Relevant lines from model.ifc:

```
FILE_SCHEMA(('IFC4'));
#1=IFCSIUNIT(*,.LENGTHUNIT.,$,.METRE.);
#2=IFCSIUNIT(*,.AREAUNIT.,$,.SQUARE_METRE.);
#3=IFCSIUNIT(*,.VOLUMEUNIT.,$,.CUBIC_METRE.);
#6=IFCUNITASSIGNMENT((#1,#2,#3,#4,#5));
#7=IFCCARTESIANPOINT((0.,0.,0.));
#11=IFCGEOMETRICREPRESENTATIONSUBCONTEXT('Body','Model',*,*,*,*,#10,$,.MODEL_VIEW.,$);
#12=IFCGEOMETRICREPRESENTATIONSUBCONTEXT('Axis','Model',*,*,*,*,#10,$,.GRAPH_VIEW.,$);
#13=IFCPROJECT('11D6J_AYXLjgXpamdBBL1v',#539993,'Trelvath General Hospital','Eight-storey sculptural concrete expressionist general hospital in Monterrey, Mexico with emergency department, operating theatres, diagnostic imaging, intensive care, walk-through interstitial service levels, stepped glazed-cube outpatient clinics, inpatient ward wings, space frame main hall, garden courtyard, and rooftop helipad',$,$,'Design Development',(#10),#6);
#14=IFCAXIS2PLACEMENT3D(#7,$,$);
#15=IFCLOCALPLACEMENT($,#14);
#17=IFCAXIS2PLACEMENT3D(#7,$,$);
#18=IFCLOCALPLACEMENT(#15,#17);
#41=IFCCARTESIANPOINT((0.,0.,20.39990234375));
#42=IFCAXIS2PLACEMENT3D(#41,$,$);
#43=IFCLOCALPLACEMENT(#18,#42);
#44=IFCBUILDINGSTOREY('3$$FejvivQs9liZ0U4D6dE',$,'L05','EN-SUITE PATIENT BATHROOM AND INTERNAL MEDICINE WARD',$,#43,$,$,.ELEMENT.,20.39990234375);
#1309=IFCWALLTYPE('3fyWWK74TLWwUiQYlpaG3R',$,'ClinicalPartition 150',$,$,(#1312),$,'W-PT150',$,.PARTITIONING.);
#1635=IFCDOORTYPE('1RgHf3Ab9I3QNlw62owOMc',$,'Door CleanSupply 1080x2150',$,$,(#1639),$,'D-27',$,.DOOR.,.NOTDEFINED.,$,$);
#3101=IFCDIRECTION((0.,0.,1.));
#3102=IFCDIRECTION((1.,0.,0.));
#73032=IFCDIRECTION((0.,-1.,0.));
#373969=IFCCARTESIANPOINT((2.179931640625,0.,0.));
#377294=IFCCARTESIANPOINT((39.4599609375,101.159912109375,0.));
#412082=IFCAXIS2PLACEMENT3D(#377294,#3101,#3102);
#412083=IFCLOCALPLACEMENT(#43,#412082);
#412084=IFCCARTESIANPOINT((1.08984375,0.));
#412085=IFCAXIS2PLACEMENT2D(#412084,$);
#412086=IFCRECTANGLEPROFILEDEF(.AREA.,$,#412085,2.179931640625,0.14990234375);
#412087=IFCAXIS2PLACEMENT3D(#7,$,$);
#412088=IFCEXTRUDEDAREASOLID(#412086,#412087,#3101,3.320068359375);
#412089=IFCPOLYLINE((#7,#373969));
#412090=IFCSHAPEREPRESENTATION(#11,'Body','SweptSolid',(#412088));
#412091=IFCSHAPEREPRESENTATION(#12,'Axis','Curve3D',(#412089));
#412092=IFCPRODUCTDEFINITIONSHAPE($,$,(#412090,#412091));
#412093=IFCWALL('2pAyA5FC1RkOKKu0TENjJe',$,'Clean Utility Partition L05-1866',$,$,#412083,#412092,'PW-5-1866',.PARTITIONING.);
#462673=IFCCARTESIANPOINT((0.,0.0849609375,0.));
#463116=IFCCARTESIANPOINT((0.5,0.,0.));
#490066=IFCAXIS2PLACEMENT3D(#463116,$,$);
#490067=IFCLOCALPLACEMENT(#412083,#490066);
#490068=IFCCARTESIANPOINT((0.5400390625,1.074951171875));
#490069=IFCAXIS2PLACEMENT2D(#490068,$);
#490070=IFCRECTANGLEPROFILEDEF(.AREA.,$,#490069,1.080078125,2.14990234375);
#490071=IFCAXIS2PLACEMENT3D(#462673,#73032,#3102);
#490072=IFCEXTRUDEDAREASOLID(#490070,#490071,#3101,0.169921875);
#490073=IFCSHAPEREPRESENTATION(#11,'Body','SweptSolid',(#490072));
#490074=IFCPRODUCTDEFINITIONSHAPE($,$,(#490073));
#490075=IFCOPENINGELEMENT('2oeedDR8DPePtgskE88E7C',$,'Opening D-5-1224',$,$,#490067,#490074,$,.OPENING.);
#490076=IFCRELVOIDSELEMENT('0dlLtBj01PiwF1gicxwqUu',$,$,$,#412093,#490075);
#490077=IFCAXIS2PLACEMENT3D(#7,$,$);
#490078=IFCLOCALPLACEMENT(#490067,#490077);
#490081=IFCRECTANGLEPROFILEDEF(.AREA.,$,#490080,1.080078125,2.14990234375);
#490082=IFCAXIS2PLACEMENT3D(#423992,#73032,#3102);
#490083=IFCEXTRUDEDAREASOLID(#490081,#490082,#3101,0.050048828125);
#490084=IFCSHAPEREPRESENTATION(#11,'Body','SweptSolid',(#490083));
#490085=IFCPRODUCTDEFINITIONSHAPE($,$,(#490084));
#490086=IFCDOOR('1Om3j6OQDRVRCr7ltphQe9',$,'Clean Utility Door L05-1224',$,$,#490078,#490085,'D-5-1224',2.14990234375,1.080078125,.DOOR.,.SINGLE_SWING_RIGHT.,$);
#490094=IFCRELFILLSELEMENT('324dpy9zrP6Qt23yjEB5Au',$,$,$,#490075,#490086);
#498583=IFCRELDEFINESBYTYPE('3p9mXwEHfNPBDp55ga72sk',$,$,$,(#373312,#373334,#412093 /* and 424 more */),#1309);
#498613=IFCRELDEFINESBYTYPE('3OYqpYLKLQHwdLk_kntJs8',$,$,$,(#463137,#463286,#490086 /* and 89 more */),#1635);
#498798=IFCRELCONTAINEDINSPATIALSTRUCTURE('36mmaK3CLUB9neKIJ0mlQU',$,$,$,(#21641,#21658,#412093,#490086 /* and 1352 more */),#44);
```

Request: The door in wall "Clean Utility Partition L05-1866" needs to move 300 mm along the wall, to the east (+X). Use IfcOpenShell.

```python
import ifcopenshell
import ifcopenshell.api.geometry
import ifcopenshell.util.placement

model = ifcopenshell.open("model.ifc")

door = model.by_guid("1Om3j6OQDRVRCr7ltphQe9")
opening = door.FillsVoids[0].RelatingOpeningElement
wall = opening.VoidsElements[0].RelatingBuildingElement

wall_matrix = ifcopenshell.util.placement.get_local_placement(wall.ObjectPlacement)
shift = wall_matrix[:3, 0] * 0.3
before = ifcopenshell.util.placement.get_local_placement(door.ObjectPlacement)[:3, 3].copy()

# The door is placed relative to its opening, so it follows when the opening moves.
matrix = ifcopenshell.util.placement.get_local_placement(opening.ObjectPlacement)
matrix[:3, 3] += shift
ifcopenshell.api.geometry.edit_object_placement(
    model, product=opening, matrix=matrix, is_si=False, should_transform_children=True
)

after = ifcopenshell.util.placement.get_local_placement(door.ObjectPlacement)[:3, 3]
print("door moved by", (after - before).round(3) + 0.0)

model.write("model-out.ifc")
```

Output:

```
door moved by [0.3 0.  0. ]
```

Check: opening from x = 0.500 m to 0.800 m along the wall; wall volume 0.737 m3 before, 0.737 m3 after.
